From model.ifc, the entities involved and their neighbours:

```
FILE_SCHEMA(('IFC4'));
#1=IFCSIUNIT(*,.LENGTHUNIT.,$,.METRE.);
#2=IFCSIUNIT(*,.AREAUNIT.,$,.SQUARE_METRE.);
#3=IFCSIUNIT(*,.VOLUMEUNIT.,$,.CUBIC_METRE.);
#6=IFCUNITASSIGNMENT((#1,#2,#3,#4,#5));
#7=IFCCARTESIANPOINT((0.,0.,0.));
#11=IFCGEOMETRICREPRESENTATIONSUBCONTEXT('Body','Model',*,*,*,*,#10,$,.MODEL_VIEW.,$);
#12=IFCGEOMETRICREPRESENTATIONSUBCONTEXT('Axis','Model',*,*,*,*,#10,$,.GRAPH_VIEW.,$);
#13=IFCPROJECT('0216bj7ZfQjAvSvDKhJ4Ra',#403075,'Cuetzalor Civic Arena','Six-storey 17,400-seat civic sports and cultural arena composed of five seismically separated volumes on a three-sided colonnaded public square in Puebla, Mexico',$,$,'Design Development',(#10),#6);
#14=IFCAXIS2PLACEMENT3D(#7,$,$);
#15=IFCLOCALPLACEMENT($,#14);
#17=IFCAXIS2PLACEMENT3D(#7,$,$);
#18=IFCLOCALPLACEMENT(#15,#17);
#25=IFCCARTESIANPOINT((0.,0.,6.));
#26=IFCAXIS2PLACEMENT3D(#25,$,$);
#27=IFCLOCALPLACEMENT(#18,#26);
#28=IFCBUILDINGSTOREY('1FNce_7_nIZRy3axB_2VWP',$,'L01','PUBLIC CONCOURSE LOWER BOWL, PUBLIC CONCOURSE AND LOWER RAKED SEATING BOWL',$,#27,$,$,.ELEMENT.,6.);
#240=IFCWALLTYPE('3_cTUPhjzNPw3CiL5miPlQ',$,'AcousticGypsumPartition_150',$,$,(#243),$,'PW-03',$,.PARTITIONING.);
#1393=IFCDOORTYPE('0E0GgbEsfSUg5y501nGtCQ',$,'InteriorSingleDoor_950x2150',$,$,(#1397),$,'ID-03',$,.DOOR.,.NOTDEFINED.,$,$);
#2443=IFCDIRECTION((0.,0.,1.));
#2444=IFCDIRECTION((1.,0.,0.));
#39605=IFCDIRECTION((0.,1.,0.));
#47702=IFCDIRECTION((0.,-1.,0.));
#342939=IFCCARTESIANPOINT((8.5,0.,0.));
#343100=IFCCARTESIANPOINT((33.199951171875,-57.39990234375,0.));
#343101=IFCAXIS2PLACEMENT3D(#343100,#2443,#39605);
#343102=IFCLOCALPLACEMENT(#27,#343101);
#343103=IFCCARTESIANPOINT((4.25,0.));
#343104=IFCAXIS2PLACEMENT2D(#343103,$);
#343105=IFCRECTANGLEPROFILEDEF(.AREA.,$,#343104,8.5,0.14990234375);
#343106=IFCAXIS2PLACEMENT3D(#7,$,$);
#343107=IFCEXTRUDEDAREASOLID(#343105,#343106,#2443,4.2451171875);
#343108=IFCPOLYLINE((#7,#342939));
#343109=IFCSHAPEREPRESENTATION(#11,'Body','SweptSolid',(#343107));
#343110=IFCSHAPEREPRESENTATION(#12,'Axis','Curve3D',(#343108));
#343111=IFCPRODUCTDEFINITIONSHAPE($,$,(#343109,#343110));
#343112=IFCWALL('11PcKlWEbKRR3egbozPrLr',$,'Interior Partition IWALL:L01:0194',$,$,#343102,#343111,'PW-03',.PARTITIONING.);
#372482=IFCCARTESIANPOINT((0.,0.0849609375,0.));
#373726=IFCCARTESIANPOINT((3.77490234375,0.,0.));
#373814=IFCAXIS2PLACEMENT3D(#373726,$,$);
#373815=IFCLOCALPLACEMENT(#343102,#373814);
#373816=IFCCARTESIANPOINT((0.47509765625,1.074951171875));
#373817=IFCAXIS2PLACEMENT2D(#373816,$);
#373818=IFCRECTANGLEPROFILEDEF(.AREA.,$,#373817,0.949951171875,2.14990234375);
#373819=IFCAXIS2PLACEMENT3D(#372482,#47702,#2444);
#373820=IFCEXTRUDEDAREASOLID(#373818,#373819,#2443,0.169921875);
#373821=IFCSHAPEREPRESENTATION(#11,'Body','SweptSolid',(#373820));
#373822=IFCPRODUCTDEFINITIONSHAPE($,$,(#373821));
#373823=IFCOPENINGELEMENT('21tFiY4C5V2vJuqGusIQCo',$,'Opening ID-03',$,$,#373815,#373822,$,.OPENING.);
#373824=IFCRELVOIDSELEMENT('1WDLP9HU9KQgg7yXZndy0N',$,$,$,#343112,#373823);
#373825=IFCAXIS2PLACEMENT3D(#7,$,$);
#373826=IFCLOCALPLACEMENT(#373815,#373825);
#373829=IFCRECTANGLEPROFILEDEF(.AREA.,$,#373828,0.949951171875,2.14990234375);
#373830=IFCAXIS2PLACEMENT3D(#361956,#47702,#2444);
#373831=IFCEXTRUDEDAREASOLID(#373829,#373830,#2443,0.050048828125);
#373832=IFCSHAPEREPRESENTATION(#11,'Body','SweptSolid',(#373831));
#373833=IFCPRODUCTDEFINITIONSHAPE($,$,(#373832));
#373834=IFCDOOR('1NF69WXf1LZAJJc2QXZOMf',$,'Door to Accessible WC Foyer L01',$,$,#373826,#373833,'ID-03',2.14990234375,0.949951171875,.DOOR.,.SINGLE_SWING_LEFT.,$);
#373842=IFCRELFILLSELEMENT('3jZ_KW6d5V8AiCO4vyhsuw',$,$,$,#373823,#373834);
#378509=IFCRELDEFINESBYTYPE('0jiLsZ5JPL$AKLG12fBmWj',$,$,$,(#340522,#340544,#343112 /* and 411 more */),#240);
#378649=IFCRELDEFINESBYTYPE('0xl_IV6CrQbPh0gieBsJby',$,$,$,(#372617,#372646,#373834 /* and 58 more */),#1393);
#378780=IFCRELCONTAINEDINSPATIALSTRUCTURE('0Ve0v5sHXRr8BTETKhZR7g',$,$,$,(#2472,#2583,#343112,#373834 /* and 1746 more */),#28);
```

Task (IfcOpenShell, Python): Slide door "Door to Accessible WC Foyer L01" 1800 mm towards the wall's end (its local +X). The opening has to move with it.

```python
import ifcopenshell
import ifcopenshell.api.geometry
import ifcopenshell.util.placement

model = ifcopenshell.open("model.ifc")

door = model.by_guid("1NF69WXf1LZAJJc2QXZOMf")
opening = door.FillsVoids[0].RelatingOpeningElement
wall = opening.VoidsElements[0].RelatingBuildingElement

wall_matrix = ifcopenshell.util.placement.get_local_placement(wall.ObjectPlacement)
shift = wall_matrix[:3, 0] * 1.8
before = ifcopenshell.util.placement.get_local_placement(door.ObjectPlacement)[:3, 3].copy()

# The door is placed relative to its opening, so it follows when the opening moves.
matrix = ifcopenshell.util.placement.get_local_placement(opening.ObjectPlacement)
matrix[:3, 3] += shift
ifcopenshell.api.geometry.edit_object_placement(
    model, product=opening, matrix=matrix, is_si=False, should_transform_children=True
)

after = ifcopenshell.util.placement.get_local_placement(door.ObjectPlacement)[:3, 3]
print("door moved by", (after - before).round(3) + 0.0)

model.write("model_updated.ifc")
```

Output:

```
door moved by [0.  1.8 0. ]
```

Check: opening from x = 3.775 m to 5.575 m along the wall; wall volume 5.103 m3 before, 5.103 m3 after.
